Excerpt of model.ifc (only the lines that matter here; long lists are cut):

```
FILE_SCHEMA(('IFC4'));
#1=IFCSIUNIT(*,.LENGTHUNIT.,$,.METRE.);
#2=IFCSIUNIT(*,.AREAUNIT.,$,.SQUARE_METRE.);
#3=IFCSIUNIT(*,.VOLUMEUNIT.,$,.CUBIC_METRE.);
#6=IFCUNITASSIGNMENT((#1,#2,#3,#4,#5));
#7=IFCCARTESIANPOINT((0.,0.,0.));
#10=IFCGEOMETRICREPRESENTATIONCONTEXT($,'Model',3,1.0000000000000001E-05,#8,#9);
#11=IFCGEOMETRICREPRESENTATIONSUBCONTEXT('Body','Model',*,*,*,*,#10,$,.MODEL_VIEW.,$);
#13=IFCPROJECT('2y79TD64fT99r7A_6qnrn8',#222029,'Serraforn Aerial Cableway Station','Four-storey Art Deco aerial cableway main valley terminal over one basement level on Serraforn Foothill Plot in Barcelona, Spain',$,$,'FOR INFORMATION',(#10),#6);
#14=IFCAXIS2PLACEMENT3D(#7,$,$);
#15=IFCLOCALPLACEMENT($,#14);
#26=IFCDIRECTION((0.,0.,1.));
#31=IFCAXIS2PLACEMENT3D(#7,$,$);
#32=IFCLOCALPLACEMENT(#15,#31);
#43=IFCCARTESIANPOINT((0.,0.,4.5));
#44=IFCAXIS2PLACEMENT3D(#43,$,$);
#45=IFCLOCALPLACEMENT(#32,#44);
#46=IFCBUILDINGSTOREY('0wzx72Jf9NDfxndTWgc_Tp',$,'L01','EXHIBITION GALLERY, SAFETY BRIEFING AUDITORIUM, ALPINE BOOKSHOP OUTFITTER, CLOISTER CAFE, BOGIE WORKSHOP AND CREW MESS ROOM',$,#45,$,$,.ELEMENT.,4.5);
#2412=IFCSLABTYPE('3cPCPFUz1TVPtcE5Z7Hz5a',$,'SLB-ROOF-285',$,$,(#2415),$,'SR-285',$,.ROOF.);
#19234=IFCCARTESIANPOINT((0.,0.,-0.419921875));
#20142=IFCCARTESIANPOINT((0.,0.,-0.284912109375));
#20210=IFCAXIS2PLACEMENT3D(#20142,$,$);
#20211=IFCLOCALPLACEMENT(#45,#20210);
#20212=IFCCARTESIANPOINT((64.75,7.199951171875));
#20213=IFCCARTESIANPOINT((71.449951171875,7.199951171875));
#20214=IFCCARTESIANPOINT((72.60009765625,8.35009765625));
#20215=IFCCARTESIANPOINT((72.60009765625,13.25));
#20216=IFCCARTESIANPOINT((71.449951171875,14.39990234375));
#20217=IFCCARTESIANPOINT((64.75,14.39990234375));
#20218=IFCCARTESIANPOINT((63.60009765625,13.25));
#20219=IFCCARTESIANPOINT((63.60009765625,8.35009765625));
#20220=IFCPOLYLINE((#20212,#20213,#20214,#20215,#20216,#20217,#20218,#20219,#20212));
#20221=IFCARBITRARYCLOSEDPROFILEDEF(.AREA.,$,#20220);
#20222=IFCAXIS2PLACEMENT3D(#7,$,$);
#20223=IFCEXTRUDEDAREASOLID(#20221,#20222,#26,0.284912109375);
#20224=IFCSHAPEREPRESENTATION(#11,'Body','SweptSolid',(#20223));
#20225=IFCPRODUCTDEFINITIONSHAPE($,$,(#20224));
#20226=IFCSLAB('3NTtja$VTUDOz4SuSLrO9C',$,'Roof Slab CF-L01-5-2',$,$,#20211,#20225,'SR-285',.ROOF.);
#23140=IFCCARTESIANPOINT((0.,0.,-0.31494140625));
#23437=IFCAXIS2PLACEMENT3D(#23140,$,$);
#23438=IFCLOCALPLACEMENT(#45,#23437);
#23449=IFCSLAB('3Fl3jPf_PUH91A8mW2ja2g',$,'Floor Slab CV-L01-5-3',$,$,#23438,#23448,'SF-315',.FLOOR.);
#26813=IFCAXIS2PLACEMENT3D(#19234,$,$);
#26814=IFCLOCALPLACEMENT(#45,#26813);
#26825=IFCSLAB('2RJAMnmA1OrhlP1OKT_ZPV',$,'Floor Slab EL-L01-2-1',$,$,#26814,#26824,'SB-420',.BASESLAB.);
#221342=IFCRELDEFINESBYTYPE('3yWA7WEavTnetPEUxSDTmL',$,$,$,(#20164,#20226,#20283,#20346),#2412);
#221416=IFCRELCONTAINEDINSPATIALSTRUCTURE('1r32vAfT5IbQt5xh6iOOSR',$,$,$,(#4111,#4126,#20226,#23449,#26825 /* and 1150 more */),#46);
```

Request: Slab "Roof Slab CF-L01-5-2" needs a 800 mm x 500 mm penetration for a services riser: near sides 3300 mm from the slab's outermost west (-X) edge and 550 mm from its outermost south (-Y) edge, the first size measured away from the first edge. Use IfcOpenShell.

```python
import numpy as np
import ifcopenshell
import ifcopenshell.api.feature
import ifcopenshell.api.geometry
import ifcopenshell.api.root
import ifcopenshell.geom
import ifcopenshell.util.placement
import ifcopenshell.util.representation
import ifcopenshell.util.shape
import ifcopenshell.util.unit

model = ifcopenshell.open("model.ifc")
unit_scale = ifcopenshell.util.unit.calculate_unit_scale(model)
settings = ifcopenshell.geom.settings()


def volume(element):
    """Net volume in cubic metres, openings subtracted."""
    shape = ifcopenshell.geom.create_shape(settings, element)
    return ifcopenshell.util.shape.get_volume(shape.geometry)


slab = model.by_guid("3NTtja$VTUDOz4SuSLrO9C")
before = volume(slab)

# Extent in the slab's own axes, in metres. The edges named are its -X and -Y sides.
slab_shape = ifcopenshell.geom.create_shape(settings, slab)
vertices = ifcopenshell.util.shape.get_vertices(slab_shape.geometry)
x_min, y_min, bottom = vertices.min(axis=0)
top = vertices[:, 2].max()

opening = ifcopenshell.api.root.create_entity(model, ifc_class="IfcOpeningElement", name="Services riser opening", predefined_type="OPENING")
context = ifcopenshell.util.representation.get_context(model, "Model", "Body", "MODEL_VIEW")
width, depth = 0.8, 0.5
outline = [(0.0, 0.0), (width, 0.0), (width, depth), (0.0, depth), (0.0, 0.0)]
# Overshoot both faces by 50 mm so the cut is clean.
shape = ifcopenshell.api.geometry.add_slab_representation(
    model, context=context, depth=top - bottom + 0.1, polyline=outline
)
ifcopenshell.api.geometry.assign_representation(model, product=opening, representation=shape)

matrix = ifcopenshell.util.placement.get_local_placement(slab.ObjectPlacement)
matrix[:, 3] = matrix @ np.append(np.array([x_min + 3.3, y_min + 0.55, bottom - 0.05]) / unit_scale, 1.0)
ifcopenshell.api.geometry.edit_object_placement(model, product=opening, matrix=matrix, is_si=False)
ifcopenshell.api.feature.add_feature(model, feature=opening, element=slab)

after = volume(slab)

print(f"slab volume {before:.3f} -> {after:.3f} m3")

model.write("model_updated.ifc")
```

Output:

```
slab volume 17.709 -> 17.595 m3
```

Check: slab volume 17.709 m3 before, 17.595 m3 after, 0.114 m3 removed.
